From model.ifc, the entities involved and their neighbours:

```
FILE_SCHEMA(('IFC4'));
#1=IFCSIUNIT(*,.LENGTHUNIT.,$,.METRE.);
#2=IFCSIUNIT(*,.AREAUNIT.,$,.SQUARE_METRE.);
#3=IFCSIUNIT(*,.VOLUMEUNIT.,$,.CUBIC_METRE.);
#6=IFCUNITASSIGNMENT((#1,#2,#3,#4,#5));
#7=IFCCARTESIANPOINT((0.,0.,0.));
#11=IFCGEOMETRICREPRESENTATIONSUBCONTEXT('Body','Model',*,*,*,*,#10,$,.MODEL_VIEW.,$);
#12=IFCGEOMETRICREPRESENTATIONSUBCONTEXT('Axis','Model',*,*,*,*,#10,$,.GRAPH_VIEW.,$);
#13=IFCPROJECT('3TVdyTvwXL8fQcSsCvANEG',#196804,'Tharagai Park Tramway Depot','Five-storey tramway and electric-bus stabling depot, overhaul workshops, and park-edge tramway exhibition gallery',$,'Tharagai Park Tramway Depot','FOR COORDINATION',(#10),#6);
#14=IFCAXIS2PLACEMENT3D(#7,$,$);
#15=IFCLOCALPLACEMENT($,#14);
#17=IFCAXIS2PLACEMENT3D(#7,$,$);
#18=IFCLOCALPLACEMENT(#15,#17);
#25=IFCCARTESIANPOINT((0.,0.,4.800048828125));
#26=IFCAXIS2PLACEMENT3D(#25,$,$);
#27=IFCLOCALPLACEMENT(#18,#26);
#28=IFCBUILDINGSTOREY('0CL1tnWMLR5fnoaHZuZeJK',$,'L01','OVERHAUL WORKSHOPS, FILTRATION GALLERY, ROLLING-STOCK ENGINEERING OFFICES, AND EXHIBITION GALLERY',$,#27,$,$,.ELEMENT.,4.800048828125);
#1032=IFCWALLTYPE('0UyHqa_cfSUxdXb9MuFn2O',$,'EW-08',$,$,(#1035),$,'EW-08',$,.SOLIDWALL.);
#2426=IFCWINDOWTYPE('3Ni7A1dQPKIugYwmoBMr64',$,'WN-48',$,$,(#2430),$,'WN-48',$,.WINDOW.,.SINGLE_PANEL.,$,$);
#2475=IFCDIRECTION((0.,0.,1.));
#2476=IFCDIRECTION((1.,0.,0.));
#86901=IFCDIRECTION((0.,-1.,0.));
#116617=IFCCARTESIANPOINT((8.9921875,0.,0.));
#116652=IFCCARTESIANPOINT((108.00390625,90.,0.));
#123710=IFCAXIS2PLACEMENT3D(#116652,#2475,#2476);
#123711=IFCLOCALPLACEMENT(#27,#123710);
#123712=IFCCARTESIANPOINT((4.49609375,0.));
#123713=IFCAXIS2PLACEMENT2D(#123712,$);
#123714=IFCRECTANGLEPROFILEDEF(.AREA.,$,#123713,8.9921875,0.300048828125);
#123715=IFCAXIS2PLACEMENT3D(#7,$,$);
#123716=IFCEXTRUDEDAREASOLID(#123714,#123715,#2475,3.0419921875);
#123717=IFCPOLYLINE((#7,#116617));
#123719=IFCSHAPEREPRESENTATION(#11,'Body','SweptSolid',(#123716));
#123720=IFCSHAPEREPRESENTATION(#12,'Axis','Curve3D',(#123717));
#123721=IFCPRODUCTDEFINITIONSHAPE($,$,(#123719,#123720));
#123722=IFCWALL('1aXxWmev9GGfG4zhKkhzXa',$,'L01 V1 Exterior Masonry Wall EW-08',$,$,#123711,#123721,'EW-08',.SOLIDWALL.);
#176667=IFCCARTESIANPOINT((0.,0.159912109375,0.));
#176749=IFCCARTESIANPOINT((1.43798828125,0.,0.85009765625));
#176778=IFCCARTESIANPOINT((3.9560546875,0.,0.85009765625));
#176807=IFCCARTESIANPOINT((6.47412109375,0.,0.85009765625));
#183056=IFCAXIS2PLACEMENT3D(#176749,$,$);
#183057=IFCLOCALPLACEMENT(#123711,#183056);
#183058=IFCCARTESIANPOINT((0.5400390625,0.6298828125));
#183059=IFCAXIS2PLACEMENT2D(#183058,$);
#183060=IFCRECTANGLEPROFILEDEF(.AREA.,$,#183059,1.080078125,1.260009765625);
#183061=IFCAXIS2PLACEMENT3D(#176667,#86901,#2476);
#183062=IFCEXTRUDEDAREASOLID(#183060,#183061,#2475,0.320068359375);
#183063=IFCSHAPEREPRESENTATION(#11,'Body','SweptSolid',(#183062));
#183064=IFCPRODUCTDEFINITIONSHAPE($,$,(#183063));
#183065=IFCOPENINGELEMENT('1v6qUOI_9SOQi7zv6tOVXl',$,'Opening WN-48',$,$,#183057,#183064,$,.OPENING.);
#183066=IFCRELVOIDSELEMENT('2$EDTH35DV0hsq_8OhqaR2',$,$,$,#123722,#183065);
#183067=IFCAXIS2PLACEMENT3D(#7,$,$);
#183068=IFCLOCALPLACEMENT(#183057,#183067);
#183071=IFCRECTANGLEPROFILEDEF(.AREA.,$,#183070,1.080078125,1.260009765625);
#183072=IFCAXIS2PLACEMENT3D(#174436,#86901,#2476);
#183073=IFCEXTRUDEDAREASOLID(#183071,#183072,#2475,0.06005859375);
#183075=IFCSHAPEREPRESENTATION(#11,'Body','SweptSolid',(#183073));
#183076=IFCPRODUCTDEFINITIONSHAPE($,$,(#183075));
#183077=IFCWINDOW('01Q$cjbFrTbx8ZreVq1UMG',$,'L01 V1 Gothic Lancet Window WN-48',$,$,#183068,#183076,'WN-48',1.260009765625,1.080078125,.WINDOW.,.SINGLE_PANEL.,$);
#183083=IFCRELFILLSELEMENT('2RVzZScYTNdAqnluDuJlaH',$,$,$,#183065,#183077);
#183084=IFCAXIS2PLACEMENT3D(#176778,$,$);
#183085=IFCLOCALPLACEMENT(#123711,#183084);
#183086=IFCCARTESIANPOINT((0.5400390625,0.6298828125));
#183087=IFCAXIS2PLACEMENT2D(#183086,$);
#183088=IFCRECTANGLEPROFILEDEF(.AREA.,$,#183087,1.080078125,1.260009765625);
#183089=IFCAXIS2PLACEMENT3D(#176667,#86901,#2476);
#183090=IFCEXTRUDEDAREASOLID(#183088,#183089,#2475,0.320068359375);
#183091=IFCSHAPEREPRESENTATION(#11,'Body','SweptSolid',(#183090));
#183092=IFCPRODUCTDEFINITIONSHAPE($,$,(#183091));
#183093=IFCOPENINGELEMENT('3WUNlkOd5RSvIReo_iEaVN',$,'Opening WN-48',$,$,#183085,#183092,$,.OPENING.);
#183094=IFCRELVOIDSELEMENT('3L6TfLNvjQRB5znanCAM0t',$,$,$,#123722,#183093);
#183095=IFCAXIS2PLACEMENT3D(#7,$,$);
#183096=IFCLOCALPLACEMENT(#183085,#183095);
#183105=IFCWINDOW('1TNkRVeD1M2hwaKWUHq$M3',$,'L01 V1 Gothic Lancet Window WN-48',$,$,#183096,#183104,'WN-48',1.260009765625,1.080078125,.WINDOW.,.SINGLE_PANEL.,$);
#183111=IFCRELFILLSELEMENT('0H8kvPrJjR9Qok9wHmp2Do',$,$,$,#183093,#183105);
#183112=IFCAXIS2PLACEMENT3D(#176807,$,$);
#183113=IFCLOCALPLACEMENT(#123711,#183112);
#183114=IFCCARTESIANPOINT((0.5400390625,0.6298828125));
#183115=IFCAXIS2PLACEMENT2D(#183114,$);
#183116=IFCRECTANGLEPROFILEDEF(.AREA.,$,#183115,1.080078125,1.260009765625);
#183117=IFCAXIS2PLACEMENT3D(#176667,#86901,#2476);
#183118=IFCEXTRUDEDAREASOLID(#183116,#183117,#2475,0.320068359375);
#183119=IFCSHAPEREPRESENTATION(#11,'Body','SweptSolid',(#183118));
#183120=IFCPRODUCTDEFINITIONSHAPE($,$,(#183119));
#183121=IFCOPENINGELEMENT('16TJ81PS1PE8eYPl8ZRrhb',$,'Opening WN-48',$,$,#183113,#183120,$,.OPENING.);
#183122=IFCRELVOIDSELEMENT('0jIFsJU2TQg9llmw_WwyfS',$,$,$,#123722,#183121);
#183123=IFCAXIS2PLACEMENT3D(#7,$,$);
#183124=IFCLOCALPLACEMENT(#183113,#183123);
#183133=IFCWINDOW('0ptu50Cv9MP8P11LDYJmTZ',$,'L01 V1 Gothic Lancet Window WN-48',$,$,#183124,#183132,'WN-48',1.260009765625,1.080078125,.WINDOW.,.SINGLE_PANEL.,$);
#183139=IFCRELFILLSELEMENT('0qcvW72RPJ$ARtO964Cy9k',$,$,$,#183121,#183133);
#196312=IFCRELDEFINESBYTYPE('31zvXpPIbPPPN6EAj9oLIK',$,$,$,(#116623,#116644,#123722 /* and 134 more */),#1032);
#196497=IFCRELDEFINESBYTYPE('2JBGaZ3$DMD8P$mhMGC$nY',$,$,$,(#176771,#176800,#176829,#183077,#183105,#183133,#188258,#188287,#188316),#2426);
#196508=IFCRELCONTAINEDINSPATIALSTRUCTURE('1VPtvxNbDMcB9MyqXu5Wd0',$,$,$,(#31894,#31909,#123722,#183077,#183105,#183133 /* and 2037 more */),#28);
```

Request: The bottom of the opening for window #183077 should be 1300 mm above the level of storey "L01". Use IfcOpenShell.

```python
import numpy as np
import ifcopenshell
import ifcopenshell.api.geometry
import ifcopenshell.geom
import ifcopenshell.util.element
import ifcopenshell.util.placement
import ifcopenshell.util.shape
import ifcopenshell.util.unit

model = ifcopenshell.open("model.ifc")
unit_scale = ifcopenshell.util.unit.calculate_unit_scale(model)

window = model.by_id(183077)
opening = window.FillsVoids[0].RelatingOpeningElement
storey = ifcopenshell.util.element.get_container(window, ifc_class="IfcBuildingStorey")
level = ifcopenshell.util.placement.get_local_placement(storey.ObjectPlacement)[2, 3]

# The opening's origin need not be at the sill, so measure its lowest point.
shape = ifcopenshell.geom.create_shape(ifcopenshell.geom.settings(), opening)
bottom = ifcopenshell.util.shape.get_shape_bottom_elevation(shape, shape.geometry) / unit_scale
dz = level + 1.3 / unit_scale - bottom

shift = np.array([0.0, 0.0, dz])
# The window is placed relative to its opening, so it follows when the opening moves.
matrix = ifcopenshell.util.placement.get_local_placement(opening.ObjectPlacement)
matrix[:3, 3] += shift
ifcopenshell.api.geometry.edit_object_placement(
    model, product=opening, matrix=matrix, is_si=False, should_transform_children=True
)

print(f"moved by {dz * unit_scale:+.3f} m")

model.write("model_rev.ifc")
```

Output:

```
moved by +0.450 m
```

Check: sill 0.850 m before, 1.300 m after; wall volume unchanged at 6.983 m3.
